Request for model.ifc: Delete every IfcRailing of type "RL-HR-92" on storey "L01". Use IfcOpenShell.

First a look at what the model holds.

```python
import ifcopenshell
import ifcopenshell.util.element

model = ifcopenshell.open("model.ifc")
print(model.schema)
storey = next(s for s in model.by_type("IfcBuildingStorey") if s.Name == "L01")
railings = [e for e in ifcopenshell.util.element.get_decomposition(storey) if e.is_a("IfcRailing")]
seen = {}
for e in railings:
    element_type = ifcopenshell.util.element.get_type(e)
    name = element_type.Name if element_type not in (None, e) else None
    seen[name] = seen.get(name, 0) + 1
for name, count in sorted(seen.items(), key=str):
    print(count, "x", name)
```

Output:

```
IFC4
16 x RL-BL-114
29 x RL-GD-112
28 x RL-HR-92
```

```python
import ifcopenshell
import ifcopenshell.api.root
import ifcopenshell.util.element

model = ifcopenshell.open("model.ifc")

storey = next(s for s in model.by_type("IfcBuildingStorey") if s.Name == "L01")
railings = [e for e in ifcopenshell.util.element.get_decomposition(storey) if e.is_a("IfcRailing")]
targets = [e for e in railings if (t := ifcopenshell.util.element.get_type(e)) not in (None, e) and t.Name == "RL-HR-92"]

for e in targets:
    ifcopenshell.api.root.remove_product(model, product=e)
print(len(targets), "removed")

model.write("model_v2.ifc")
```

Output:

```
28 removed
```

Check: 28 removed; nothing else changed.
